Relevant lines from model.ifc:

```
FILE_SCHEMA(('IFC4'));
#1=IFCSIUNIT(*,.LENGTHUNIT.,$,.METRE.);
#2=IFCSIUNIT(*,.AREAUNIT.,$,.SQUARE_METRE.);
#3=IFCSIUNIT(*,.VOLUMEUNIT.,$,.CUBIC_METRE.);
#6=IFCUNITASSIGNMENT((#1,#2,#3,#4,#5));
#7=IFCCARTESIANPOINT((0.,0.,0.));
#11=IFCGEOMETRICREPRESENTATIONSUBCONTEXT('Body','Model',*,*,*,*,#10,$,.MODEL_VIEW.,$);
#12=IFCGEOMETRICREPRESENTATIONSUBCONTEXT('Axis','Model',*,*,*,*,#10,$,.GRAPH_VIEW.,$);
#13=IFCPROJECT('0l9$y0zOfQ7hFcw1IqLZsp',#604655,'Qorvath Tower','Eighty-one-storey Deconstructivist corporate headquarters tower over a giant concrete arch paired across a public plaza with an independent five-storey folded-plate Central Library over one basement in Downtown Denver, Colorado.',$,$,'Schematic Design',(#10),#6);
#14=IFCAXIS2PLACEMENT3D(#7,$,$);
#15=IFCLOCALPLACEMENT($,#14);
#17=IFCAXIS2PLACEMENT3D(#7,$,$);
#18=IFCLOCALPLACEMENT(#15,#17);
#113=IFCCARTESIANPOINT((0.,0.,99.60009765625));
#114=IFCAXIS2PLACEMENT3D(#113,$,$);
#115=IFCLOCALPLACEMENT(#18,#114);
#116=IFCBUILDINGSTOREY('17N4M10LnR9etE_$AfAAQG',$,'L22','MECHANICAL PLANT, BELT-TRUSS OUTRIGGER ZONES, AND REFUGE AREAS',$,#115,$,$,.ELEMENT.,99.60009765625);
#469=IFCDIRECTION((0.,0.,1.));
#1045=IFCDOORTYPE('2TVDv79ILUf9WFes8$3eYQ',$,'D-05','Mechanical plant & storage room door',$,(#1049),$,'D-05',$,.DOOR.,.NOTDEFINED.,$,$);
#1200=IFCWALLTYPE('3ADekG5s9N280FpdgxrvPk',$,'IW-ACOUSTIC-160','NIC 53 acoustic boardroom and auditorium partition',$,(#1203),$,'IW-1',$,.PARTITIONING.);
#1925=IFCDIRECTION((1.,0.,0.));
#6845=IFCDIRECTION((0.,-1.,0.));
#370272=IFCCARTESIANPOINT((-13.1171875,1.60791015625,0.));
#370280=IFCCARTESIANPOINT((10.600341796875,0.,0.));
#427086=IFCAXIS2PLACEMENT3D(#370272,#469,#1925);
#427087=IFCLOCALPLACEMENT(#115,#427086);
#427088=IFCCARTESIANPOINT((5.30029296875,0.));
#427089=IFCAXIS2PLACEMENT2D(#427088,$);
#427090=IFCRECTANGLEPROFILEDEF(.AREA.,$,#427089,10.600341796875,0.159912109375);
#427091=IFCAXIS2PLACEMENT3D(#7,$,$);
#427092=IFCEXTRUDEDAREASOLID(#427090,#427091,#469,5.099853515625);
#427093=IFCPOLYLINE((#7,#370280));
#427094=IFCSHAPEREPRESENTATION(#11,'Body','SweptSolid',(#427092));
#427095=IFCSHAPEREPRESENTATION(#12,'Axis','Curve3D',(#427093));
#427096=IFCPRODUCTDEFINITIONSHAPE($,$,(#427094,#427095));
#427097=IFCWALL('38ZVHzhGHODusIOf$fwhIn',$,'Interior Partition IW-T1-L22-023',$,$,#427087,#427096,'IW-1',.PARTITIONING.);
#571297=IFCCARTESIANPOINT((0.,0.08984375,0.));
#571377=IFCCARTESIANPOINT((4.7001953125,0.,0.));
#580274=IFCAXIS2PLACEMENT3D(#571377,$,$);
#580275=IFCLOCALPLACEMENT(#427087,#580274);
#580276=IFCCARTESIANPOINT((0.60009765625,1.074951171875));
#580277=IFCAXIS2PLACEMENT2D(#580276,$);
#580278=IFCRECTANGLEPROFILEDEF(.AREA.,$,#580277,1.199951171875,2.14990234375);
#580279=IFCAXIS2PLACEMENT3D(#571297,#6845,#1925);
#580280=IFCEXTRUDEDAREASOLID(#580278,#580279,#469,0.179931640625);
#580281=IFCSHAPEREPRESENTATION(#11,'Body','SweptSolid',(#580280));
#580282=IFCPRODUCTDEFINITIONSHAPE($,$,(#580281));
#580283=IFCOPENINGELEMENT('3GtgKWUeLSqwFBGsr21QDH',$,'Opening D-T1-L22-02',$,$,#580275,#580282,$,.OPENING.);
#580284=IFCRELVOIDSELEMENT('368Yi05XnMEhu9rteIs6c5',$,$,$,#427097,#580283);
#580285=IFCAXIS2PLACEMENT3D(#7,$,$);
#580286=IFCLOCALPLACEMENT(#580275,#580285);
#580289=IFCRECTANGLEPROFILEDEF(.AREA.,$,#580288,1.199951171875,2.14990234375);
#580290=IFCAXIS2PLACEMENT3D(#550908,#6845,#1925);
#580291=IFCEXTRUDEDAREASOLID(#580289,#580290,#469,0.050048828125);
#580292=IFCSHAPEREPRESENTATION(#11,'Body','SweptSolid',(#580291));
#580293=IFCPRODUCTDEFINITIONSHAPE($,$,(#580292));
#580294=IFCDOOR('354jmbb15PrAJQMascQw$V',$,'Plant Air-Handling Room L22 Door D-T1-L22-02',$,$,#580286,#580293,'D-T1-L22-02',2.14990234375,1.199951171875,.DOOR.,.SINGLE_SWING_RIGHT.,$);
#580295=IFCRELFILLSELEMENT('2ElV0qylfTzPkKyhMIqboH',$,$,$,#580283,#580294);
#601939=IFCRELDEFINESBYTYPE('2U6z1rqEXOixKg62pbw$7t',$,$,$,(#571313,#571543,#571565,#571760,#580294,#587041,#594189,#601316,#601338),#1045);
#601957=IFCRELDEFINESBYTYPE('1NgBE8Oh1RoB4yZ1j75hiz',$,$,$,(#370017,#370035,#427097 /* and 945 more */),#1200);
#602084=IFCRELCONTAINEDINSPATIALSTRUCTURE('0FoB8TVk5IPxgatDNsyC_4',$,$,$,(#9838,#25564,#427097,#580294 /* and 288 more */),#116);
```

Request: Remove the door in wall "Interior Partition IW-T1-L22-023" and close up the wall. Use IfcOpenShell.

```python
import ifcopenshell
import ifcopenshell.api.feature
import ifcopenshell.api.root
import ifcopenshell.geom
import ifcopenshell.util.shape

model = ifcopenshell.open("model.ifc")
settings = ifcopenshell.geom.settings()


def volume(element):
    """Net volume in cubic metres, openings subtracted."""
    shape = ifcopenshell.geom.create_shape(settings, element)
    return ifcopenshell.util.shape.get_volume(shape.geometry)


door = model.by_id(580294)
opening = door.FillsVoids[0].RelatingOpeningElement
wall = opening.VoidsElements[0].RelatingBuildingElement
before = volume(wall)

ifcopenshell.api.root.remove_product(model, product=door)
ifcopenshell.api.feature.remove_feature(model, feature=opening)

after = volume(wall)

print(f"wall volume {before:.3f} -> {after:.3f} m3")

model.write("model_edited.ifc")
```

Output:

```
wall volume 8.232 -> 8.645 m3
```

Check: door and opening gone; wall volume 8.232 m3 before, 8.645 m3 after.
